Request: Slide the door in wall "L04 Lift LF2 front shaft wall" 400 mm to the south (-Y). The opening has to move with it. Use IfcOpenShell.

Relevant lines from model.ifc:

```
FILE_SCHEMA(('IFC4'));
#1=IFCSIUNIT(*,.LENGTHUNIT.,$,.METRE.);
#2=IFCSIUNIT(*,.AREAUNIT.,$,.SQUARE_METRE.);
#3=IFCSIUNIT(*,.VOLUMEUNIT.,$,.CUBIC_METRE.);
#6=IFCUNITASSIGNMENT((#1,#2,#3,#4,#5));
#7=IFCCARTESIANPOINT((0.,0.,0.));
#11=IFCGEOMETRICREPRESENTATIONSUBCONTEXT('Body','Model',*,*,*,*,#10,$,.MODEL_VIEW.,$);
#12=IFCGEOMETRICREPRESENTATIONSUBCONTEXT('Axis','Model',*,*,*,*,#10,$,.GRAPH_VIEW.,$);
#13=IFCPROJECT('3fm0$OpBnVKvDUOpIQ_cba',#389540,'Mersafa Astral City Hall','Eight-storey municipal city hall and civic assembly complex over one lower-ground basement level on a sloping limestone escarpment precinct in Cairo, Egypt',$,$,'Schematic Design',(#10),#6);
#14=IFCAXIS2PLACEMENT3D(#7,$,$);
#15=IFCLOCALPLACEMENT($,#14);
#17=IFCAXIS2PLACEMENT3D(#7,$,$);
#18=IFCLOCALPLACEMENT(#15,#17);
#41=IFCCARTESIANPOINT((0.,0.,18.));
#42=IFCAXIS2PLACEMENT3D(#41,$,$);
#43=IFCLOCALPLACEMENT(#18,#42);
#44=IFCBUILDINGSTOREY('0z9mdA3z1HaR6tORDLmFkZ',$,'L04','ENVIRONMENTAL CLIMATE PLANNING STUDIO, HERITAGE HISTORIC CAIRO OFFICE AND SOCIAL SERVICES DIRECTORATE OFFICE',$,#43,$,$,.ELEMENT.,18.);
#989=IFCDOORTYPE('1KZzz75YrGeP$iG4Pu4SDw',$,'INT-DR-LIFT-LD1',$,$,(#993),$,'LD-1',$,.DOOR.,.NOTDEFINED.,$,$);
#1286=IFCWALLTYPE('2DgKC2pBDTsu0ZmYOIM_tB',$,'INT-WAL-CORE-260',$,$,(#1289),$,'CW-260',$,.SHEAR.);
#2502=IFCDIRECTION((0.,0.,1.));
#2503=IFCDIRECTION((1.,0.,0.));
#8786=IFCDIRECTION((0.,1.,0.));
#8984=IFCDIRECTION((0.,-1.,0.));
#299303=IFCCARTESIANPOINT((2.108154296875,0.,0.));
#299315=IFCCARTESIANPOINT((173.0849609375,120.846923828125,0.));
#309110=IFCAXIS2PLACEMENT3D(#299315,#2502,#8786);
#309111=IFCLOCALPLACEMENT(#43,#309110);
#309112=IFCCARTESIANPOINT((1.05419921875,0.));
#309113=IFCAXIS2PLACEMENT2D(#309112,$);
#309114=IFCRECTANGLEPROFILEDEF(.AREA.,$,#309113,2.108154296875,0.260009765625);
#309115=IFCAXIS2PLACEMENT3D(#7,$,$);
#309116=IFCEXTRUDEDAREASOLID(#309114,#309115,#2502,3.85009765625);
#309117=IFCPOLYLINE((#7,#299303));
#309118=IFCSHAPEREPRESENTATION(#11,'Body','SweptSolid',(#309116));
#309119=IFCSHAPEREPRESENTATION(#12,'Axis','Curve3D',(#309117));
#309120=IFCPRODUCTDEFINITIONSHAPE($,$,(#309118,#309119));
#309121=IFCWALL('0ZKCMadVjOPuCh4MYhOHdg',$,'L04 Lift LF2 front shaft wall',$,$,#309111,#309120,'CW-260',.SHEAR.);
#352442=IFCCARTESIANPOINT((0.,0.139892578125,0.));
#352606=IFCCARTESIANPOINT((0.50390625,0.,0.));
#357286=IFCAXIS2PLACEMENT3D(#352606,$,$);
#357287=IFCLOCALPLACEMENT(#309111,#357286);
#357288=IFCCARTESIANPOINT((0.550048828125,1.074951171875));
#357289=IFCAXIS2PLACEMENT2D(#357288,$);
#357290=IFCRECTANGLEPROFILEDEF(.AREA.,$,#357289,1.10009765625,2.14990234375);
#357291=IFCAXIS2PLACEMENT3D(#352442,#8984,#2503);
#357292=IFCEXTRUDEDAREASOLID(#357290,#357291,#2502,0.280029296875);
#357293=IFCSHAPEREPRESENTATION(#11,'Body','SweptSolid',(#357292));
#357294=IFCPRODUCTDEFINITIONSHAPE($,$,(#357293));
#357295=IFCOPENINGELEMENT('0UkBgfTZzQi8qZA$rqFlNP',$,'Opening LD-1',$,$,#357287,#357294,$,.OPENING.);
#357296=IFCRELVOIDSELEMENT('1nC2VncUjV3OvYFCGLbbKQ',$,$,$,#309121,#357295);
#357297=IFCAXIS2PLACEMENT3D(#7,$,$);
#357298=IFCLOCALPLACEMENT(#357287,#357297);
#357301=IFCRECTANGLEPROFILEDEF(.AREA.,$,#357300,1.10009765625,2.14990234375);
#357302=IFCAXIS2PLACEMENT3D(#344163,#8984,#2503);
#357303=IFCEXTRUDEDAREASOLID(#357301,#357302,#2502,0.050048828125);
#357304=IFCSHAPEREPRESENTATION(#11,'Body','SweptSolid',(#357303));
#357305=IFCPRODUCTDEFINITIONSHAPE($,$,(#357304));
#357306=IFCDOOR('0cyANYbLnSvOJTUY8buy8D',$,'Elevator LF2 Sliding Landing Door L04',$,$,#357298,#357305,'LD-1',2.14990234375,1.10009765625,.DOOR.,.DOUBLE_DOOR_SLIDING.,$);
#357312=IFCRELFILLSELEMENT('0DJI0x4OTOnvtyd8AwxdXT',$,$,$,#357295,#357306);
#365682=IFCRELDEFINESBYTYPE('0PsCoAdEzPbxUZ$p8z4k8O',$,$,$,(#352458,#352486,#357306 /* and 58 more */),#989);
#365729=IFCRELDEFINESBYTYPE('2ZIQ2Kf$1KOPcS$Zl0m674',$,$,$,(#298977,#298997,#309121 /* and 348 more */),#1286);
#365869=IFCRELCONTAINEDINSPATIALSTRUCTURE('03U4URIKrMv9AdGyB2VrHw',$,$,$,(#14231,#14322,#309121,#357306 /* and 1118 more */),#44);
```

```python
import ifcopenshell
import ifcopenshell.api.geometry
import ifcopenshell.util.placement

model = ifcopenshell.open("model.ifc")

door = model.by_guid("0cyANYbLnSvOJTUY8buy8D")
opening = door.FillsVoids[0].RelatingOpeningElement
wall = opening.VoidsElements[0].RelatingBuildingElement

wall_matrix = ifcopenshell.util.placement.get_local_placement(wall.ObjectPlacement)
shift = wall_matrix[:3, 0] * -0.4
before = ifcopenshell.util.placement.get_local_placement(door.ObjectPlacement)[:3, 3].copy()

# The door is placed relative to its opening, so it follows when the opening moves.
matrix = ifcopenshell.util.placement.get_local_placement(opening.ObjectPlacement)
matrix[:3, 3] += shift
ifcopenshell.api.geometry.edit_object_placement(
    model, product=opening, matrix=matrix, is_si=False, should_transform_children=True
)

after = ifcopenshell.util.placement.get_local_placement(door.ObjectPlacement)[:3, 3]
print("door moved by", (after - before).round(3) + 0.0)

model.write("model_rev.ifc")
```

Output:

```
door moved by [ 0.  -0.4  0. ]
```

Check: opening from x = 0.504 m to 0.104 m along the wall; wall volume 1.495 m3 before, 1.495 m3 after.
